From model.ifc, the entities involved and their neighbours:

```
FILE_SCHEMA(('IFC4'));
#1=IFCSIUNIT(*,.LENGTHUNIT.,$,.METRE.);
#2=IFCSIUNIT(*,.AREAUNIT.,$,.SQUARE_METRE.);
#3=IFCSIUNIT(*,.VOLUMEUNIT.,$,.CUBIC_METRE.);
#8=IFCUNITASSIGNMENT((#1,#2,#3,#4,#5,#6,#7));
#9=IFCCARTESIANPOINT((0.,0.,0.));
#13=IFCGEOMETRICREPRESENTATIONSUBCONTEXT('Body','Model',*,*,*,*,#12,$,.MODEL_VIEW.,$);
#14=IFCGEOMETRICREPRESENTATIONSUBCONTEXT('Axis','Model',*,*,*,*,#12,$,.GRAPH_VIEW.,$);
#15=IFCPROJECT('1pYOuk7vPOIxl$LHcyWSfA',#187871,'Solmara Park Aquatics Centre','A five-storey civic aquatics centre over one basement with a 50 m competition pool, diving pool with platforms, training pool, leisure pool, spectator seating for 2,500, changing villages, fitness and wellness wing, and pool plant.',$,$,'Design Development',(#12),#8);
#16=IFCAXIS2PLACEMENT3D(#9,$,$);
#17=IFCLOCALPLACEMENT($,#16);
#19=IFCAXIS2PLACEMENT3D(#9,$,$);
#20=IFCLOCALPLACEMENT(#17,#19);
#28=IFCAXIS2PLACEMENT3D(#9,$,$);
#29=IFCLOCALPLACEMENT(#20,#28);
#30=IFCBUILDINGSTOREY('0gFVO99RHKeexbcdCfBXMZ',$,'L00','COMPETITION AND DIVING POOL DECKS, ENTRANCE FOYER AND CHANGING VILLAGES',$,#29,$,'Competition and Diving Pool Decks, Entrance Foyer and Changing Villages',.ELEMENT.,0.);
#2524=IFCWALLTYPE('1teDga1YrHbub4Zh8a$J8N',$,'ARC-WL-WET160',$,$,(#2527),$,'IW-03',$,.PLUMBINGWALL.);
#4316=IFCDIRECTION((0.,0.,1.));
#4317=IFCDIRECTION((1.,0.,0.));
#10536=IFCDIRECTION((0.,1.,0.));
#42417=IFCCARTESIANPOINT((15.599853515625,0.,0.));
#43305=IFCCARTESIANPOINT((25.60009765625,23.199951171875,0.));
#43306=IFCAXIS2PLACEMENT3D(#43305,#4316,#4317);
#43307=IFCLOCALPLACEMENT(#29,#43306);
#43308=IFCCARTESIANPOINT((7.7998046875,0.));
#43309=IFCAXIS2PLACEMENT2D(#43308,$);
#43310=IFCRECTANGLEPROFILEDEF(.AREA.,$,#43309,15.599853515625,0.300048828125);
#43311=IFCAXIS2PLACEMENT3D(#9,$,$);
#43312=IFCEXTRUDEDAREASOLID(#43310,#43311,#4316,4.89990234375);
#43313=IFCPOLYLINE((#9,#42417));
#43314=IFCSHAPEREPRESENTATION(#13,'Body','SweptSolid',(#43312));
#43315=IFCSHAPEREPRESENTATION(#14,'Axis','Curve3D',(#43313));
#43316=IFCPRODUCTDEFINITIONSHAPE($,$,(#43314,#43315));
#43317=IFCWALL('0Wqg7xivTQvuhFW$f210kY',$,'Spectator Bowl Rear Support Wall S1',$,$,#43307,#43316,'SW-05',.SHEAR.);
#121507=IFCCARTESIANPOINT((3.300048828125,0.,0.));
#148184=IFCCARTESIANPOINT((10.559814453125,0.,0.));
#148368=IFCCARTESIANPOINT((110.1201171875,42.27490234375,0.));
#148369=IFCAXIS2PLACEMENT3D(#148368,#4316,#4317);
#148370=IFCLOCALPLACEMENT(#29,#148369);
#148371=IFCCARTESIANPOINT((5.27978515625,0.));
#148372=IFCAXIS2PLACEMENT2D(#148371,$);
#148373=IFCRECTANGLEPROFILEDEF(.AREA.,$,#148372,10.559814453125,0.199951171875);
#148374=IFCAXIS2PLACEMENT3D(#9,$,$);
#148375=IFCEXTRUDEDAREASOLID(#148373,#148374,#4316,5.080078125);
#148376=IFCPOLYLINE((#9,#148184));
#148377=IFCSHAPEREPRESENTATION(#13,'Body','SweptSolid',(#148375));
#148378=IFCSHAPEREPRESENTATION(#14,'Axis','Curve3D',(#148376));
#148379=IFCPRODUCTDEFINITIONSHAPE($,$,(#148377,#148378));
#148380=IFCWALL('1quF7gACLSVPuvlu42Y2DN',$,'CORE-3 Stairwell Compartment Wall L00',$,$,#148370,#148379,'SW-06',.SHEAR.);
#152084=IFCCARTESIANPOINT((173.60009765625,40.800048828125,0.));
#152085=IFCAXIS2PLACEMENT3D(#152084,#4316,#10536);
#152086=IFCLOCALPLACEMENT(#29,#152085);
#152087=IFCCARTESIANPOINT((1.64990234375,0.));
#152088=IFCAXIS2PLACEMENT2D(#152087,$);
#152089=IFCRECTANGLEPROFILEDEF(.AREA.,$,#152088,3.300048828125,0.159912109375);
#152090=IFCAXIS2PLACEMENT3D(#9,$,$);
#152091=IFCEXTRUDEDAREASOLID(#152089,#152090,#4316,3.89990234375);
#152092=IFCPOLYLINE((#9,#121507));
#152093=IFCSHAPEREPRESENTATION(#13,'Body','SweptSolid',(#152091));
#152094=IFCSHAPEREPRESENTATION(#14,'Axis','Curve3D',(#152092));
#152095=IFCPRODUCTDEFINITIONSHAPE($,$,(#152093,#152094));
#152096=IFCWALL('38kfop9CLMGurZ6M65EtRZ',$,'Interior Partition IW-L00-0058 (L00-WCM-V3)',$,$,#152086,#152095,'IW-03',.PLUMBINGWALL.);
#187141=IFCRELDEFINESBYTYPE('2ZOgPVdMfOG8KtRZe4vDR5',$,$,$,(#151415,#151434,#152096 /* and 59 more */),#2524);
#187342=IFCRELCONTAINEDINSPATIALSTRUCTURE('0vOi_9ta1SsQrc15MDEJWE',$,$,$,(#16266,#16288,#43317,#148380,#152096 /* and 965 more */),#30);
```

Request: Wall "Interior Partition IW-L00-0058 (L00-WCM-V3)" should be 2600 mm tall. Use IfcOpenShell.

```python
import ifcopenshell
import ifcopenshell.geom
import ifcopenshell.util.representation
import ifcopenshell.util.shape

model = ifcopenshell.open("model.ifc")
settings = ifcopenshell.geom.settings()


def volume(element):
    """Net volume in cubic metres, openings subtracted."""
    shape = ifcopenshell.geom.create_shape(settings, element)
    return ifcopenshell.util.shape.get_volume(shape.geometry)


wall = model.by_guid("38kfop9CLMGurZ6M65EtRZ")
before = volume(wall)

body = ifcopenshell.util.representation.get_representation(wall, "Model", "Body")
solid = body.Items[0]
old_height = solid.Depth
solid.Depth = 2.6
after = volume(wall)

print(f"height {old_height:g} -> {solid.Depth:g}, volume {before:.3f} -> {after:.3f} m3")

model.write("model_v2.ifc")
```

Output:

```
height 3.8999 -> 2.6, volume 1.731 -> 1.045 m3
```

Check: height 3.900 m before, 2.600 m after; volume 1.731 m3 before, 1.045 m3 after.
